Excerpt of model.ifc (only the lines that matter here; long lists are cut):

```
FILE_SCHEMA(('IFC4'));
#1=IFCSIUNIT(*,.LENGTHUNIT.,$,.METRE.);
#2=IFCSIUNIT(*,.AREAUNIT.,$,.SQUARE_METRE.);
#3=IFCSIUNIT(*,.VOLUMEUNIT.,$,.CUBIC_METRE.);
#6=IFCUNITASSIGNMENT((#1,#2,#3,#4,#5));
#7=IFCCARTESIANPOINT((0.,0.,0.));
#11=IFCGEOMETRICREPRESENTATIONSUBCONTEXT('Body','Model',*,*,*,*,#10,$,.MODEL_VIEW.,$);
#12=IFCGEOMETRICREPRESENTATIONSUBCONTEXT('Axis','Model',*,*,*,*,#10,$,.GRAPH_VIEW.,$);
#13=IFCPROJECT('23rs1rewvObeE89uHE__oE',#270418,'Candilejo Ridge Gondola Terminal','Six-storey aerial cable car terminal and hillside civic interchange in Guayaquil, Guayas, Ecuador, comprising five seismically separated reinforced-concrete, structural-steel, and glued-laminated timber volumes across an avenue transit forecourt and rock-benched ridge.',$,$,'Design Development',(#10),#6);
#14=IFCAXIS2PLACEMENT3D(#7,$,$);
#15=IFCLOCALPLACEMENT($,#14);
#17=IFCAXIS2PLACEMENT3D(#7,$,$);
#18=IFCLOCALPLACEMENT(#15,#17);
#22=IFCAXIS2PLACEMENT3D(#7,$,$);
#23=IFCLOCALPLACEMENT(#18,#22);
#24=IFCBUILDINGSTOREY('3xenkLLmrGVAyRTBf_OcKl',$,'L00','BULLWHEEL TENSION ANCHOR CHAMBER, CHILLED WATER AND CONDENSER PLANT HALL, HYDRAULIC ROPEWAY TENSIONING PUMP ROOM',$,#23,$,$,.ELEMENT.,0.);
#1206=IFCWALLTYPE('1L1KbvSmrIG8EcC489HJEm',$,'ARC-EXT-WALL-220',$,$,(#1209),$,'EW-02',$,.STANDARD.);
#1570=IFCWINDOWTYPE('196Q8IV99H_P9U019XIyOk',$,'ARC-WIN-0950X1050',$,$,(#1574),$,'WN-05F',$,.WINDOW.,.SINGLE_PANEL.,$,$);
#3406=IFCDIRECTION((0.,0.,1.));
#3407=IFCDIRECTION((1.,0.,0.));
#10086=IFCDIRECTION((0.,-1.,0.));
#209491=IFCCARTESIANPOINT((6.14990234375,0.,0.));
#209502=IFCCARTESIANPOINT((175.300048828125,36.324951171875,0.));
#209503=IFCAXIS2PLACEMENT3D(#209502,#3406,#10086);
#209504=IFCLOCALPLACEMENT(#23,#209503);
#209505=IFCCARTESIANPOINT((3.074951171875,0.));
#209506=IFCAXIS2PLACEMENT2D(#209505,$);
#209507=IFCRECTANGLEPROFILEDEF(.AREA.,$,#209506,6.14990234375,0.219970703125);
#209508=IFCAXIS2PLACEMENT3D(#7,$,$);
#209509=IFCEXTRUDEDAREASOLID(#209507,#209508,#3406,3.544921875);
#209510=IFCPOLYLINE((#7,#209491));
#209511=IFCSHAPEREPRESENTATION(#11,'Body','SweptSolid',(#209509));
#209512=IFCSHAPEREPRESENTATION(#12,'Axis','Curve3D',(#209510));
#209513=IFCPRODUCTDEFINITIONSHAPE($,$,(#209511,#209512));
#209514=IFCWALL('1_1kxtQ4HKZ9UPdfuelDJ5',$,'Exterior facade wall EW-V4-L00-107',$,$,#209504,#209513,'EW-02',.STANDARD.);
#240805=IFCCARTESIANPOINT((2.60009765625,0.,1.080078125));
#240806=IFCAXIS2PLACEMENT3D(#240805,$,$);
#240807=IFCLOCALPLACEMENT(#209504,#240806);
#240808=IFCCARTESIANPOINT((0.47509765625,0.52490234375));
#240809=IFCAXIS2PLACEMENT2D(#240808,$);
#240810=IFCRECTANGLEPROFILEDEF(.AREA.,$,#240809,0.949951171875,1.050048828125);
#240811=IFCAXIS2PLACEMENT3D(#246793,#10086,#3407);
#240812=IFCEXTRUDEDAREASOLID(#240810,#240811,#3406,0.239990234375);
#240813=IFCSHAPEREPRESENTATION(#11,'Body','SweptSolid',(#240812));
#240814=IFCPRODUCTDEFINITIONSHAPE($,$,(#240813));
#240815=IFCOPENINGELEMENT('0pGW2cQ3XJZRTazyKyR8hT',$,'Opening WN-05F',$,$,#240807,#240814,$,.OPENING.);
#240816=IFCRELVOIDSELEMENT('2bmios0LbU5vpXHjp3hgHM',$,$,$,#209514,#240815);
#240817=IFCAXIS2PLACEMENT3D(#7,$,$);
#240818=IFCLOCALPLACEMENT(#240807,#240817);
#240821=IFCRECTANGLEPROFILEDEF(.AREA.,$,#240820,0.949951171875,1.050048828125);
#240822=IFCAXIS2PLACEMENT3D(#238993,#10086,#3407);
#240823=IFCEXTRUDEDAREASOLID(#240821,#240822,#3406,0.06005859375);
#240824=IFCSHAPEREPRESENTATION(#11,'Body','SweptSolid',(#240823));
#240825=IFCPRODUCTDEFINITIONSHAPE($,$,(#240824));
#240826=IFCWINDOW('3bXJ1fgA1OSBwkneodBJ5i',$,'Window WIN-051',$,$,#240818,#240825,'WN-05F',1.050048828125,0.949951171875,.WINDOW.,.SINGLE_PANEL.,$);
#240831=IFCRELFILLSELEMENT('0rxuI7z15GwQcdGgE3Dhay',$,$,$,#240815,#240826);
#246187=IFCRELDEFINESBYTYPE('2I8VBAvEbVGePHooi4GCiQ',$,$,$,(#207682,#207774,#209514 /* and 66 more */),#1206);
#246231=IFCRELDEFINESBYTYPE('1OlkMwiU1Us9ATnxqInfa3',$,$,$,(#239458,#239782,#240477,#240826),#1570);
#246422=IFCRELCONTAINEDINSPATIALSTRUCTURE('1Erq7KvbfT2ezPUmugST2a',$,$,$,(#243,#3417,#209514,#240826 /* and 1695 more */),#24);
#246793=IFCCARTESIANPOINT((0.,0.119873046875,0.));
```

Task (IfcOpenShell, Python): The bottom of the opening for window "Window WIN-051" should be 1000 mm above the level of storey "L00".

```python
import numpy as np
import ifcopenshell
import ifcopenshell.api.geometry
import ifcopenshell.geom
import ifcopenshell.util.element
import ifcopenshell.util.placement
import ifcopenshell.util.shape
import ifcopenshell.util.unit

model = ifcopenshell.open("model.ifc")
unit_scale = ifcopenshell.util.unit.calculate_unit_scale(model)

window = model.by_guid("3bXJ1fgA1OSBwkneodBJ5i")
opening = window.FillsVoids[0].RelatingOpeningElement
storey = ifcopenshell.util.element.get_container(window, ifc_class="IfcBuildingStorey")
level = ifcopenshell.util.placement.get_local_placement(storey.ObjectPlacement)[2, 3]

# The opening's origin need not be at the sill, so measure its lowest point.
shape = ifcopenshell.geom.create_shape(ifcopenshell.geom.settings(), opening)
bottom = ifcopenshell.util.shape.get_shape_bottom_elevation(shape, shape.geometry) / unit_scale
dz = level + 1 / unit_scale - bottom

shift = np.array([0.0, 0.0, dz])
# The window is placed relative to its opening, so it follows when the opening moves.
matrix = ifcopenshell.util.placement.get_local_placement(opening.ObjectPlacement)
matrix[:3, 3] += shift
ifcopenshell.api.geometry.edit_object_placement(
    model, product=opening, matrix=matrix, is_si=False, should_transform_children=True
)

print(f"moved by {dz * unit_scale:+.3f} m")

model.write("model-out.ifc")
```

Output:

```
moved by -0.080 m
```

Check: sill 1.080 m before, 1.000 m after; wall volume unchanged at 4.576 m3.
